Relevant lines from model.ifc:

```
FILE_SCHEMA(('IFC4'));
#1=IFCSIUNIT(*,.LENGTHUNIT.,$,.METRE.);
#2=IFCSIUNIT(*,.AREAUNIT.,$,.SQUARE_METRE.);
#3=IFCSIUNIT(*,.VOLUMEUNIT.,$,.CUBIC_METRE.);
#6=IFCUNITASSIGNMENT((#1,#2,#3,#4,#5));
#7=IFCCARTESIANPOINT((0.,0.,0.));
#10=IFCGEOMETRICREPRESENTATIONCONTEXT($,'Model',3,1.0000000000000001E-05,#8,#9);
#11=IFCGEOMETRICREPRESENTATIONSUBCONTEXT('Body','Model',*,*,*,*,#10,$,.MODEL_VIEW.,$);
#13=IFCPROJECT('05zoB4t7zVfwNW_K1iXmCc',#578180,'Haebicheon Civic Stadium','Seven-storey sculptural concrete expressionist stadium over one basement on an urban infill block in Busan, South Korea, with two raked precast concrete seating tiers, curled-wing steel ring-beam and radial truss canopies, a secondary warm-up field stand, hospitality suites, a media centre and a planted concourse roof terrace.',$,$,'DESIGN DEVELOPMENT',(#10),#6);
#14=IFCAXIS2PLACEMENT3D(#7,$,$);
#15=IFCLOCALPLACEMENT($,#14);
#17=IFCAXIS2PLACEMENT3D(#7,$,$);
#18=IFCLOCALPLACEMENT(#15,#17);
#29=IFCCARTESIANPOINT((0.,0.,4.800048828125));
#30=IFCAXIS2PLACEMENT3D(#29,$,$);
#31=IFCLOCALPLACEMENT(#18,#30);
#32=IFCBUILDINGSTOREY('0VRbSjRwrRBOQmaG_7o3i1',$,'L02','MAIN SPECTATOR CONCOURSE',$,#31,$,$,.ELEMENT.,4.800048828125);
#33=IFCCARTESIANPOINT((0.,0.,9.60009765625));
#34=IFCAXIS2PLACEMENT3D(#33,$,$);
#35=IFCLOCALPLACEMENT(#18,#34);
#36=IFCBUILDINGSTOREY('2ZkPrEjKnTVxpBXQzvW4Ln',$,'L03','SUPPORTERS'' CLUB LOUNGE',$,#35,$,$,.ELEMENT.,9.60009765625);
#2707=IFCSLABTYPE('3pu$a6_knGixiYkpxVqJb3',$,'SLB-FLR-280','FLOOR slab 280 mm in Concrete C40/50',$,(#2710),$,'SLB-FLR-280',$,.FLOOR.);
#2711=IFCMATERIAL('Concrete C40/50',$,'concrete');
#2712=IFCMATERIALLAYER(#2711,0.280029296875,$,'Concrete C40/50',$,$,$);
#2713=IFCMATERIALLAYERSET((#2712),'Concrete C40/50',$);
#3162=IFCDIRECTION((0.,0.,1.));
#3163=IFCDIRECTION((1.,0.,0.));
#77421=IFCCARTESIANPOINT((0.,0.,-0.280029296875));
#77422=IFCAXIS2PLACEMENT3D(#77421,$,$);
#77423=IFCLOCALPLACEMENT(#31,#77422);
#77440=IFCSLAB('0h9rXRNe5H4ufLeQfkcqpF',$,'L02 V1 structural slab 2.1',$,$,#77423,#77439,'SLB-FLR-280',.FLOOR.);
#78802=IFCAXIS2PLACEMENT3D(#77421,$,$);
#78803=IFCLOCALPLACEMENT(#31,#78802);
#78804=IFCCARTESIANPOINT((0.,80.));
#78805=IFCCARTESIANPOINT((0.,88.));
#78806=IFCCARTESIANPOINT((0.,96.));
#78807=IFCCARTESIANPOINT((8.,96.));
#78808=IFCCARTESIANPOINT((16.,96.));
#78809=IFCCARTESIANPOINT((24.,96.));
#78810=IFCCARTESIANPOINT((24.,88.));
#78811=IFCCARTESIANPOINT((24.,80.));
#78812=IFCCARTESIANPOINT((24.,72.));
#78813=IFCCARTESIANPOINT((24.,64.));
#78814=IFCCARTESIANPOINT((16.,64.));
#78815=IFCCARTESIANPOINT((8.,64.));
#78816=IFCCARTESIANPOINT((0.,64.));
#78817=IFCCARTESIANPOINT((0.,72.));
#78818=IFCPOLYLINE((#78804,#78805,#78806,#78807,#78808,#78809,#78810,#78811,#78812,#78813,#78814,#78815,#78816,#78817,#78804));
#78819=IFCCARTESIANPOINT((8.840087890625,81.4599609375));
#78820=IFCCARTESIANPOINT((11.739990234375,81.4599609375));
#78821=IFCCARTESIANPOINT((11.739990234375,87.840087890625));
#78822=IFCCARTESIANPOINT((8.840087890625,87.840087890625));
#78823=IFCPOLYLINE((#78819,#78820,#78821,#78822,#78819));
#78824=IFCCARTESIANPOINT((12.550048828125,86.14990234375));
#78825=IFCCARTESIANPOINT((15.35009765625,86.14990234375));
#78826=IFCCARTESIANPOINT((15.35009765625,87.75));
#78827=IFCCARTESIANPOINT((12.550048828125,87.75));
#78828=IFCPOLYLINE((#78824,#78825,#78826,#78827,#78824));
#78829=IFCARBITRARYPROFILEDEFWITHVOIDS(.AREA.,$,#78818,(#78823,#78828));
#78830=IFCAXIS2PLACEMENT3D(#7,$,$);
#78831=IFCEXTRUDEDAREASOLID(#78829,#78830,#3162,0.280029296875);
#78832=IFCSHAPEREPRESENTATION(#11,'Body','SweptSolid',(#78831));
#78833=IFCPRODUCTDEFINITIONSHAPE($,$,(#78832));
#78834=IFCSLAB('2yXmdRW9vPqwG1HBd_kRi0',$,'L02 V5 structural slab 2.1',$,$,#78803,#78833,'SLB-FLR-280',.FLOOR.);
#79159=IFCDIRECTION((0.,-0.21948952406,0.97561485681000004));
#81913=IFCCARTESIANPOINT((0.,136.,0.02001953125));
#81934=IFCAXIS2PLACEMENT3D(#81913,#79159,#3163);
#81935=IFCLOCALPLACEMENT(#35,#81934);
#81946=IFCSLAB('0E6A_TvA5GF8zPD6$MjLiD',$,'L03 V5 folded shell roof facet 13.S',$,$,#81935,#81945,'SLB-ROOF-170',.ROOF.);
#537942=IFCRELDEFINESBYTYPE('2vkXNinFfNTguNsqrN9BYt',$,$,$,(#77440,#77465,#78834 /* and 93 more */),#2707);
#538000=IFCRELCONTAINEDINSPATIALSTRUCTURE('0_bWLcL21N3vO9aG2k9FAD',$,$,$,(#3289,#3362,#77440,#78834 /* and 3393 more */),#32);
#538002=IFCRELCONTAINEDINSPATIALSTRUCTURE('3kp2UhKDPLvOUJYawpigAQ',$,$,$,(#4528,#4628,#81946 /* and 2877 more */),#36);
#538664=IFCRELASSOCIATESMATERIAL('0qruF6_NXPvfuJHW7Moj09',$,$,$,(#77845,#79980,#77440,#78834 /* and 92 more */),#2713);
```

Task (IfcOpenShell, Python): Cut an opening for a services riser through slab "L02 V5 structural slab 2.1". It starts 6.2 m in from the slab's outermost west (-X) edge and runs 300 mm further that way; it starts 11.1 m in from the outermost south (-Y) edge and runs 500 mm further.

```python
import numpy as np
import ifcopenshell
import ifcopenshell.api.feature
import ifcopenshell.api.geometry
import ifcopenshell.api.root
import ifcopenshell.geom
import ifcopenshell.util.placement
import ifcopenshell.util.representation
import ifcopenshell.util.shape
import ifcopenshell.util.unit

model = ifcopenshell.open("model.ifc")
unit_scale = ifcopenshell.util.unit.calculate_unit_scale(model)
settings = ifcopenshell.geom.settings()


def volume(element):
    """Net volume in cubic metres, openings subtracted."""
    shape = ifcopenshell.geom.create_shape(settings, element)
    return ifcopenshell.util.shape.get_volume(shape.geometry)


slab = model.by_guid("2yXmdRW9vPqwG1HBd_kRi0")
before = volume(slab)

# Extent in the slab's own axes, in metres. The edges named are its -X and -Y sides.
slab_shape = ifcopenshell.geom.create_shape(settings, slab)
vertices = ifcopenshell.util.shape.get_vertices(slab_shape.geometry)
x_min, y_min, bottom = vertices.min(axis=0)
top = vertices[:, 2].max()

opening = ifcopenshell.api.root.create_entity(model, ifc_class="IfcOpeningElement", name="Services riser opening", predefined_type="OPENING")
context = ifcopenshell.util.representation.get_context(model, "Model", "Body", "MODEL_VIEW")
width, depth = 0.3, 0.5
outline = [(0.0, 0.0), (width, 0.0), (width, depth), (0.0, depth), (0.0, 0.0)]
# Overshoot both faces by 50 mm so the cut is clean.
shape = ifcopenshell.api.geometry.add_slab_representation(
    model, context=context, depth=top - bottom + 0.1, polyline=outline
)
ifcopenshell.api.geometry.assign_representation(model, product=opening, representation=shape)

matrix = ifcopenshell.util.placement.get_local_placement(slab.ObjectPlacement)
matrix[:, 3] = matrix @ np.append(np.array([x_min + 6.2, y_min + 11.1, bottom - 0.05]) / unit_scale, 1.0)
ifcopenshell.api.geometry.edit_object_placement(model, product=opening, matrix=matrix, is_si=False)
ifcopenshell.api.feature.add_feature(model, feature=opening, element=slab)

after = volume(slab)

print(f"slab volume {before:.3f} -> {after:.3f} m3")

model.write("model-out.ifc")
```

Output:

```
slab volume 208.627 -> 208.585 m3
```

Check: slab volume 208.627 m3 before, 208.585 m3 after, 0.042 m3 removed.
